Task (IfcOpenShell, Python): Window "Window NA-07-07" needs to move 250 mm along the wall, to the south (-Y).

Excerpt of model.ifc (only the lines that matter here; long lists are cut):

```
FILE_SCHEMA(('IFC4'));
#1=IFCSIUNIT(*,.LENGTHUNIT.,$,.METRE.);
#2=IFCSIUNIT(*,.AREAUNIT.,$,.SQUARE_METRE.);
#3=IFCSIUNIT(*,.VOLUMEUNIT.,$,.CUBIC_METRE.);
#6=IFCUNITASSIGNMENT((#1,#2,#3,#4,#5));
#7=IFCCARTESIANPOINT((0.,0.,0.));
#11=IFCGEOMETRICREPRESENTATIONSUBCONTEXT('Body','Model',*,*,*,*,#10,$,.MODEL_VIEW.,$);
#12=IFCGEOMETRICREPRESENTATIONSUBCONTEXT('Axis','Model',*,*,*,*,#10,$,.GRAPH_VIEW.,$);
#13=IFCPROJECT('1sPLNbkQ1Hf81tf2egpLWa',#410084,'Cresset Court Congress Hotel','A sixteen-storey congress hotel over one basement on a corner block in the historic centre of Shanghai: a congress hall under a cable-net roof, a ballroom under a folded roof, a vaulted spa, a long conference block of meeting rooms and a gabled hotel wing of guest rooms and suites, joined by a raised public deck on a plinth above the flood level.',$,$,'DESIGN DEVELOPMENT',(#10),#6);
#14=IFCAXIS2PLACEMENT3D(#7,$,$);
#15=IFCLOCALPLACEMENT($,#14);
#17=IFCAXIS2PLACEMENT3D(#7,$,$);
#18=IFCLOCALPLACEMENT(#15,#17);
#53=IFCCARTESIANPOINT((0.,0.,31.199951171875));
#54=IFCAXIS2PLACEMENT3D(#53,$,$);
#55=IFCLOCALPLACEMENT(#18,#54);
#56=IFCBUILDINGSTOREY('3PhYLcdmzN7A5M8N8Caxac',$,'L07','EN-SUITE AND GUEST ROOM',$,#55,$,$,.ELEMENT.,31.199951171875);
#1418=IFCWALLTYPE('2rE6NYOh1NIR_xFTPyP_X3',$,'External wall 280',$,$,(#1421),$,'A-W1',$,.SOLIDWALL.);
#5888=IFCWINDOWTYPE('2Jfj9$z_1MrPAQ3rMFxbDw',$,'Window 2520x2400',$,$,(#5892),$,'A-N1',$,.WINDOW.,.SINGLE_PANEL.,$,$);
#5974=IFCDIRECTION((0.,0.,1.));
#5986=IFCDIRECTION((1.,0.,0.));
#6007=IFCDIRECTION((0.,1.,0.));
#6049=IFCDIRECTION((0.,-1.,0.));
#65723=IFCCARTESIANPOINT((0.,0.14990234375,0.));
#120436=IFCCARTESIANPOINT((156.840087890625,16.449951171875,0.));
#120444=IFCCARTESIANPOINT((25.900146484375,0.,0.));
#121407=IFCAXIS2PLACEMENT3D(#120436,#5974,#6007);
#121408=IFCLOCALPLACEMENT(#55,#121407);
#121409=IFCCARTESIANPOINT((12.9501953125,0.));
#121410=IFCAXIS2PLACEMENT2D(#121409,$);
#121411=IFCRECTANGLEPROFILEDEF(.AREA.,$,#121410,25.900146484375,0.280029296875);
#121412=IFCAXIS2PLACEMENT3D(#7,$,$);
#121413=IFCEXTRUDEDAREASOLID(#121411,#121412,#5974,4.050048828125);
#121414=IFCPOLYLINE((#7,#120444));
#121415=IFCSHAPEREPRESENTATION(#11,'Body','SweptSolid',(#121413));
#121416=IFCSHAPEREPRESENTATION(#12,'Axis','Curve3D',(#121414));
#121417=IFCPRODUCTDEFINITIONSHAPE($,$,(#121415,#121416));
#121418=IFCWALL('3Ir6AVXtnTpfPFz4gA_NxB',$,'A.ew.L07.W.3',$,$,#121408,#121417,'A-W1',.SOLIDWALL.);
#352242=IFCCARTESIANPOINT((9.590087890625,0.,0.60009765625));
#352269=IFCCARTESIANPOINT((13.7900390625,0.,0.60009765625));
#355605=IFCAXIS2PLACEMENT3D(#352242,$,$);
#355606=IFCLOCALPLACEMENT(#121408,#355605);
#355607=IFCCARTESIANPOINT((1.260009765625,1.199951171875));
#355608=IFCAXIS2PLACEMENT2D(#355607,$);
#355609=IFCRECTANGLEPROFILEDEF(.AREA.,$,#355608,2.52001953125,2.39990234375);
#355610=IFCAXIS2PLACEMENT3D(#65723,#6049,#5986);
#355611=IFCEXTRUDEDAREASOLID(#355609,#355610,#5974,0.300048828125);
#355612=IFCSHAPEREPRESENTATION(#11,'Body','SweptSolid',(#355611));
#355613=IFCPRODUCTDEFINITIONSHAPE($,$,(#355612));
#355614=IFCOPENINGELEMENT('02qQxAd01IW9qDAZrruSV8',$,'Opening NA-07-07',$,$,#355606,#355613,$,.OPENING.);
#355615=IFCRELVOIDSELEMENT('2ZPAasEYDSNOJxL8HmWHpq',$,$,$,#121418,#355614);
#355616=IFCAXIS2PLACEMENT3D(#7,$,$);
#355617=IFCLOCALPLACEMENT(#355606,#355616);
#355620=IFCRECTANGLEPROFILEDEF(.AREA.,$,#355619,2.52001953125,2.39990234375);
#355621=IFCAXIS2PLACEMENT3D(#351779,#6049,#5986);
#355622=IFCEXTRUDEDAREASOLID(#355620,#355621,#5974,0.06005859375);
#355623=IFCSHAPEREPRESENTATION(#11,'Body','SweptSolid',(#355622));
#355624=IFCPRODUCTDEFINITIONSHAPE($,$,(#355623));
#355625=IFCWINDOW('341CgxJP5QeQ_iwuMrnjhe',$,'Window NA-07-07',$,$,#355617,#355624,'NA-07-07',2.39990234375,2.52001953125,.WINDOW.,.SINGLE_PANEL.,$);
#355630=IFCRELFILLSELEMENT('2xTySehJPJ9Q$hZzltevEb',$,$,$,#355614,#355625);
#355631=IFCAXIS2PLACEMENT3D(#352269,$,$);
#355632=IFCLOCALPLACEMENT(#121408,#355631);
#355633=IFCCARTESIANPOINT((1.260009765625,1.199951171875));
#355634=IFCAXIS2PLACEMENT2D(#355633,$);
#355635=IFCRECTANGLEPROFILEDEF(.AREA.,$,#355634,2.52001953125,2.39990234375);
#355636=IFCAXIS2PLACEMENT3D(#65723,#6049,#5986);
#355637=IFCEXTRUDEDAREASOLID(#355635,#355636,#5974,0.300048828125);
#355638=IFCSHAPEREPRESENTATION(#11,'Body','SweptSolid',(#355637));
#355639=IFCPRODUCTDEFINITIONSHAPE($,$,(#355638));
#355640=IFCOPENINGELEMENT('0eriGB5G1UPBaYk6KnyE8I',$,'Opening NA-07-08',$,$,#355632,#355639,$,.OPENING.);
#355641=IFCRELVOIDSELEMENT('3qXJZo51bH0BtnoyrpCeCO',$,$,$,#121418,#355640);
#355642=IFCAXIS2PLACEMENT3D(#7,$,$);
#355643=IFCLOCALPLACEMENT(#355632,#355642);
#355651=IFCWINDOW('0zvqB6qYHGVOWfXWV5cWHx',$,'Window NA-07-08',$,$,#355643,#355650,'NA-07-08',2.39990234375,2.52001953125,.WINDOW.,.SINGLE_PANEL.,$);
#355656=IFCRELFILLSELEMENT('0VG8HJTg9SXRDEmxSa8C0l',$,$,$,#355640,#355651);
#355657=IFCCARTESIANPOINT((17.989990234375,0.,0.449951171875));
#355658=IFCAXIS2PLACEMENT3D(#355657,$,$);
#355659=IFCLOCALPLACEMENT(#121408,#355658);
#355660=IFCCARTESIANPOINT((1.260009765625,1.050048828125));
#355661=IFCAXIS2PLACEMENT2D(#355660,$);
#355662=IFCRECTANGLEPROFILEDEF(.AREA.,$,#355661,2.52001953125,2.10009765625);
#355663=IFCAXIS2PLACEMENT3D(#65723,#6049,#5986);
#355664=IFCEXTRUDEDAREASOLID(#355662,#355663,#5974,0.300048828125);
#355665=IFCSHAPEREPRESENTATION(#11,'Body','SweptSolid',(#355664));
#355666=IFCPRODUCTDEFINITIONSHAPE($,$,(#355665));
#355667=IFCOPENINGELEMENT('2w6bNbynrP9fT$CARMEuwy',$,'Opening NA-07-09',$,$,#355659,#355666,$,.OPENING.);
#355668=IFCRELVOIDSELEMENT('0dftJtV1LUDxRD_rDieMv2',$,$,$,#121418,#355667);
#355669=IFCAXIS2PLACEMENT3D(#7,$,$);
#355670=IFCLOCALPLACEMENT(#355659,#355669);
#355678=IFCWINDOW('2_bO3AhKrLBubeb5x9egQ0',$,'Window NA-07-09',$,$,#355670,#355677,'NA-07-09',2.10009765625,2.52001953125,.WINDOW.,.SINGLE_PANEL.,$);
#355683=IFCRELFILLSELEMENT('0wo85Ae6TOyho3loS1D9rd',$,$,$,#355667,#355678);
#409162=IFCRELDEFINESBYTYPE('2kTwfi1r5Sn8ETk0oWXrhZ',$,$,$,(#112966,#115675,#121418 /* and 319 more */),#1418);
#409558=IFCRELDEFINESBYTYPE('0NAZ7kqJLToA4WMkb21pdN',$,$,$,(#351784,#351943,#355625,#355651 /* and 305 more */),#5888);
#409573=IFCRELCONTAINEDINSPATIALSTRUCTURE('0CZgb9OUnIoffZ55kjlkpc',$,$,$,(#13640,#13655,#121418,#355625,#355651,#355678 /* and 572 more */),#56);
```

```python
import ifcopenshell
import ifcopenshell.api.geometry
import ifcopenshell.util.placement
import ifcopenshell.util.unit

model = ifcopenshell.open("model.ifc")
unit_scale = ifcopenshell.util.unit.calculate_unit_scale(model)

window = model.by_guid("341CgxJP5QeQ_iwuMrnjhe")
opening = window.FillsVoids[0].RelatingOpeningElement
wall = opening.VoidsElements[0].RelatingBuildingElement

wall_matrix = ifcopenshell.util.placement.get_local_placement(wall.ObjectPlacement)
shift = wall_matrix[:3, 0] * -0.25 / unit_scale
before = ifcopenshell.util.placement.get_local_placement(window.ObjectPlacement)[:3, 3].copy()

# The window is placed relative to its opening, so it follows when the opening moves.
matrix = ifcopenshell.util.placement.get_local_placement(opening.ObjectPlacement)
matrix[:3, 3] += shift
ifcopenshell.api.geometry.edit_object_placement(
    model, product=opening, matrix=matrix, is_si=False, should_transform_children=True
)

after = ifcopenshell.util.placement.get_local_placement(window.ObjectPlacement)[:3, 3]
print("window moved by", (after - before).round(3) + 0.0)

model.write("model_rev.ifc")
```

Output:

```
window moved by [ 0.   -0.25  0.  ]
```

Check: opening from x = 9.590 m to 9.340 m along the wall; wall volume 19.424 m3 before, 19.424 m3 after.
